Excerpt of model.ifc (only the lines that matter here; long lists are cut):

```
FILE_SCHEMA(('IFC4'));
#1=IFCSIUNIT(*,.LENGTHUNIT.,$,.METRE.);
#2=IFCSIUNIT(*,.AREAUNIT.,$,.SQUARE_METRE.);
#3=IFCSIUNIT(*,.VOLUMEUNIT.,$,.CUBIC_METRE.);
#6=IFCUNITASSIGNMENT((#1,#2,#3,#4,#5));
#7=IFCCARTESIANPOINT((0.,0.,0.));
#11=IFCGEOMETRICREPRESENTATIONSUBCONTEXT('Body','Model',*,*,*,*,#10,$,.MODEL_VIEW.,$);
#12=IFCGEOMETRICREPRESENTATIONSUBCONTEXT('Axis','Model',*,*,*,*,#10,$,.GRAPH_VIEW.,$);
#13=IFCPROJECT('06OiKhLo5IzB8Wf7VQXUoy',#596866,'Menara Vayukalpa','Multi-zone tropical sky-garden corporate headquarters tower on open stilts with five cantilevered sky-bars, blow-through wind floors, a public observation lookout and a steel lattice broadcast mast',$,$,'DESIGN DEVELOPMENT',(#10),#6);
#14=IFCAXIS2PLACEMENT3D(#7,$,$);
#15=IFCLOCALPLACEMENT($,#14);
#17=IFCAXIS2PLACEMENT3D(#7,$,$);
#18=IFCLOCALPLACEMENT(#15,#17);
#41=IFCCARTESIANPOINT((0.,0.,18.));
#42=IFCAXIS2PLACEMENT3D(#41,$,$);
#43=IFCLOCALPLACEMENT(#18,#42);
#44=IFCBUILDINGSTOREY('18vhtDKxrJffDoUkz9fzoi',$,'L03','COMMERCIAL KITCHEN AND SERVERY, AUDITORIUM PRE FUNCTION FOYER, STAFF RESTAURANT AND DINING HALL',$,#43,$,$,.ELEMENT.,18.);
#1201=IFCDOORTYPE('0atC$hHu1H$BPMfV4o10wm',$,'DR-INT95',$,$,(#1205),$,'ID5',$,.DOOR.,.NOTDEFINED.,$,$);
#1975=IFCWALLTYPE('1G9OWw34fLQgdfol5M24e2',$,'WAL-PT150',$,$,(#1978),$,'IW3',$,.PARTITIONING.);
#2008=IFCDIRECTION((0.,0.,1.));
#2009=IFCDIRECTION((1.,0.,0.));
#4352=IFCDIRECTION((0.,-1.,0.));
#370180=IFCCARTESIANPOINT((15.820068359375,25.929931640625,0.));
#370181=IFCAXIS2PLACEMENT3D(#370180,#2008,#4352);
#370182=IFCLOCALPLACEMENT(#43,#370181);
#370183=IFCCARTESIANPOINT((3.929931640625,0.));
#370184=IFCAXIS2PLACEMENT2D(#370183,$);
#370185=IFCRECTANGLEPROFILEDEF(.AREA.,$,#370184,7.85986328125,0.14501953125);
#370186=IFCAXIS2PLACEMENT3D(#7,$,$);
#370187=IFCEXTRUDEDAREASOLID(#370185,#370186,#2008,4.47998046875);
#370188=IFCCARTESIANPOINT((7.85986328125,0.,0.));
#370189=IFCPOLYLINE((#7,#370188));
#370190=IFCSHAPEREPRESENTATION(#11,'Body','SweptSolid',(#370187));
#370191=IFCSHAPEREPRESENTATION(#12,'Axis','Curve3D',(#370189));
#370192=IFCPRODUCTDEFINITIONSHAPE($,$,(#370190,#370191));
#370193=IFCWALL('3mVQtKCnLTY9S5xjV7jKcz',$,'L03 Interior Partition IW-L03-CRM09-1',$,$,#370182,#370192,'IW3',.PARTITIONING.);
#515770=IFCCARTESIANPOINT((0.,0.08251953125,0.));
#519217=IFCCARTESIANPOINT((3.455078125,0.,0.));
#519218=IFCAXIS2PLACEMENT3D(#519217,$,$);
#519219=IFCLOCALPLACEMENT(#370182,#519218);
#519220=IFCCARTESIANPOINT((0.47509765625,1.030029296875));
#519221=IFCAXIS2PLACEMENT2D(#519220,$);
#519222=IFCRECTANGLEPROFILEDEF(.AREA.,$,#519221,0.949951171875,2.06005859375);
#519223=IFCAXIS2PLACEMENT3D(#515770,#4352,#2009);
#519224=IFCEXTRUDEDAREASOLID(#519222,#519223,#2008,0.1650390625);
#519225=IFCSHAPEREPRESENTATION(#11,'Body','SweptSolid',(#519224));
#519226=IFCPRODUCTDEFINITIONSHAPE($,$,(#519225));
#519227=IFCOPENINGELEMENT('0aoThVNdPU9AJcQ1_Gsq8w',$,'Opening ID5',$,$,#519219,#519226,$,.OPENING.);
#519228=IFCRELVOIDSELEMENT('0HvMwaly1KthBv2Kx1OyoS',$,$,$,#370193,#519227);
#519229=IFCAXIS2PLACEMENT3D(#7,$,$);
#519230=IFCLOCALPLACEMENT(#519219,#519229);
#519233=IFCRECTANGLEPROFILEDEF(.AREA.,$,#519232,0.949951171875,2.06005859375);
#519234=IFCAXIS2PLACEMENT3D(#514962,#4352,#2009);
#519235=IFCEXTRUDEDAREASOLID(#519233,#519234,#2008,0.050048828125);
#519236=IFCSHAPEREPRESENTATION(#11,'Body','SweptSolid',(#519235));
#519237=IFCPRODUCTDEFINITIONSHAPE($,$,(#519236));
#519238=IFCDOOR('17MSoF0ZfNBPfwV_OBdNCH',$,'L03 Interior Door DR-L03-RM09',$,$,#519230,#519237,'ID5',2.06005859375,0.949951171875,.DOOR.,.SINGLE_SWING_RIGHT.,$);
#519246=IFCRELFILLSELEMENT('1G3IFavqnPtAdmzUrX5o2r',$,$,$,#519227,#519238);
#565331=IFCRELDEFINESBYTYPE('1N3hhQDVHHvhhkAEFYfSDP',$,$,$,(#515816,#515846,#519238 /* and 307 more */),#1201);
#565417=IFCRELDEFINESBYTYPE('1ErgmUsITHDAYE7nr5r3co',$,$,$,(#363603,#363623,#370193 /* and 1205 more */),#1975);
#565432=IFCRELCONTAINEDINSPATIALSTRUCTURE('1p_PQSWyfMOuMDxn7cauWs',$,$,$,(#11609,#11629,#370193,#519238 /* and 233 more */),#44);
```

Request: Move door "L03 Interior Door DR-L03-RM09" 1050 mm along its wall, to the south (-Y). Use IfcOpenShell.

```python
import ifcopenshell
import ifcopenshell.api.geometry
import ifcopenshell.util.placement

model = ifcopenshell.open("model.ifc")

door = model.by_guid("17MSoF0ZfNBPfwV_OBdNCH")
opening = door.FillsVoids[0].RelatingOpeningElement
wall = opening.VoidsElements[0].RelatingBuildingElement

wall_matrix = ifcopenshell.util.placement.get_local_placement(wall.ObjectPlacement)
shift = wall_matrix[:3, 0] * 1.05
before = ifcopenshell.util.placement.get_local_placement(door.ObjectPlacement)[:3, 3].copy()

# The door is placed relative to its opening, so it follows when the opening moves.
matrix = ifcopenshell.util.placement.get_local_placement(opening.ObjectPlacement)
matrix[:3, 3] += shift
ifcopenshell.api.geometry.edit_object_placement(
    model, product=opening, matrix=matrix, is_si=False, should_transform_children=True
)

after = ifcopenshell.util.placement.get_local_placement(door.ObjectPlacement)[:3, 3]
print("door moved by", (after - before).round(3) + 0.0)

model.write("model-out.ifc")
```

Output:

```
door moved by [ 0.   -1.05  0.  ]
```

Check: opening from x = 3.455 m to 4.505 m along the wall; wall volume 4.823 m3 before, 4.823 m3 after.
